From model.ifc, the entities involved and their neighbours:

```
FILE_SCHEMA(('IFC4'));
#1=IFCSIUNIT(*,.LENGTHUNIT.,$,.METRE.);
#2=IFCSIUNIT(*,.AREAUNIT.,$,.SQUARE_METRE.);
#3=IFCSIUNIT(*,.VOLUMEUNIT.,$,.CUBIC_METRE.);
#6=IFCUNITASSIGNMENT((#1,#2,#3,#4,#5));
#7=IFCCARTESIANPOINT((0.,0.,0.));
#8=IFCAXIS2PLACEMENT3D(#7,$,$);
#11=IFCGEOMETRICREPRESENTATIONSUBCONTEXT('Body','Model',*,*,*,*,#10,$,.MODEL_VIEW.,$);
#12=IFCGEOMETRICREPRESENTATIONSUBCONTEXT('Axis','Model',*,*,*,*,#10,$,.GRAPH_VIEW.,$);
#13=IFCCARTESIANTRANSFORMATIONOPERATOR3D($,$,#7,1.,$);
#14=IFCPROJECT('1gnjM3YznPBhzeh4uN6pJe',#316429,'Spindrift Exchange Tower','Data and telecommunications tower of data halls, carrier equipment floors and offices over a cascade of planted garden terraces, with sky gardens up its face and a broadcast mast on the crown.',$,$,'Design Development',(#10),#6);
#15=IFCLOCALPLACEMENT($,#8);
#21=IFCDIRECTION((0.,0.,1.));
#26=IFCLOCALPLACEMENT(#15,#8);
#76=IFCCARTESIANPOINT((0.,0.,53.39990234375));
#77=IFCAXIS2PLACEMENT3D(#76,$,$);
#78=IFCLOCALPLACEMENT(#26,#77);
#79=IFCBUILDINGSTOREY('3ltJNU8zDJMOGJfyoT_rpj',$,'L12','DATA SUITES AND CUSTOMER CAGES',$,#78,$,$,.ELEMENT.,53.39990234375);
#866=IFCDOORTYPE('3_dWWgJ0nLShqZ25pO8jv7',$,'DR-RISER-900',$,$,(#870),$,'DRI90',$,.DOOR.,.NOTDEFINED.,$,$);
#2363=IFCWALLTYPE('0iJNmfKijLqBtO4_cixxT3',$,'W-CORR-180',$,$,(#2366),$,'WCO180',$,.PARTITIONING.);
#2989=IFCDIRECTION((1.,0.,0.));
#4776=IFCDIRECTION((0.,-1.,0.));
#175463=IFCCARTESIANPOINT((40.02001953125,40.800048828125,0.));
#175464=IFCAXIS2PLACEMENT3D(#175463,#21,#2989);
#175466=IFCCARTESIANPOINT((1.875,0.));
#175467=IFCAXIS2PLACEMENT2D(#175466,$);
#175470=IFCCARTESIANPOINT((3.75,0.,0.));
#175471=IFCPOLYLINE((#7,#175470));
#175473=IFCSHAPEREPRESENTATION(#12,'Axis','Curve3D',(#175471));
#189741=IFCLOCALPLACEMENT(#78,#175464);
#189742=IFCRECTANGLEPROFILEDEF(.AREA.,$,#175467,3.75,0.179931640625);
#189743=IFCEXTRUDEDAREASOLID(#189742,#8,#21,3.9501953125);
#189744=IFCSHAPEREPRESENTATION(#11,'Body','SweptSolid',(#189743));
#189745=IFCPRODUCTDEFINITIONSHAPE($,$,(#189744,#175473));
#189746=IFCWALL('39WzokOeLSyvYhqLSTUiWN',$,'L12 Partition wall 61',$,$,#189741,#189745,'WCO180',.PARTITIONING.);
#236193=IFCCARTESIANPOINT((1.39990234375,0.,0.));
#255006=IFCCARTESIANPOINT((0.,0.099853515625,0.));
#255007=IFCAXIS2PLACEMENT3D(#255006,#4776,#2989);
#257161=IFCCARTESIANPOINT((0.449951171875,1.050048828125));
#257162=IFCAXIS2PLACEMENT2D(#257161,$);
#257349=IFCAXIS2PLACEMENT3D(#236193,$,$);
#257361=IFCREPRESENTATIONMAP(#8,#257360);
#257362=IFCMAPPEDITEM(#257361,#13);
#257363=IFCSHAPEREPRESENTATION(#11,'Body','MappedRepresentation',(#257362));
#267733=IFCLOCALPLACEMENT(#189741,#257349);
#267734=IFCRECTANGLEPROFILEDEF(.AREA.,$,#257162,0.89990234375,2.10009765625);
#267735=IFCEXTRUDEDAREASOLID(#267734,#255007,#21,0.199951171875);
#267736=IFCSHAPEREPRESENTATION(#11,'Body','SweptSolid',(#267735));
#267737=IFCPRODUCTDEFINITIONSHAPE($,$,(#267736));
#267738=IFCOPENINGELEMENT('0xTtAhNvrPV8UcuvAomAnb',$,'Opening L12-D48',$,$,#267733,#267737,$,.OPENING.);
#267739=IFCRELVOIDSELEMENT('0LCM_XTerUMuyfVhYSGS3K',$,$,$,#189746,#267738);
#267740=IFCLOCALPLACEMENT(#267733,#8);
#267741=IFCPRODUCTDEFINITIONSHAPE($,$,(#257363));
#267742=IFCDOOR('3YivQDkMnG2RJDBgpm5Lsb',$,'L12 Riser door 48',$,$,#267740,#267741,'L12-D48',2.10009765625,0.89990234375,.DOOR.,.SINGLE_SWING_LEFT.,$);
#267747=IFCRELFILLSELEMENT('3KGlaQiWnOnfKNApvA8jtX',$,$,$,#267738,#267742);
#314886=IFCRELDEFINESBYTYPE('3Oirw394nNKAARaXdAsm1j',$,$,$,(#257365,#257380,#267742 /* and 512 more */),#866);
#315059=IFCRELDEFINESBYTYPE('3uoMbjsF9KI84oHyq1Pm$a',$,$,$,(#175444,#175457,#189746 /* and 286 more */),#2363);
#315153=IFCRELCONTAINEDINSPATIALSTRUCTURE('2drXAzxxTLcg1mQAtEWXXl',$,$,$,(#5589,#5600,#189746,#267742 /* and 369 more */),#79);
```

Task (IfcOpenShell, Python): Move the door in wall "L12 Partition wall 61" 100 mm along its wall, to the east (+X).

```python
import ifcopenshell
import ifcopenshell.api.geometry
import ifcopenshell.util.placement

model = ifcopenshell.open("model.ifc")

door = model.by_guid("3YivQDkMnG2RJDBgpm5Lsb")
opening = door.FillsVoids[0].RelatingOpeningElement
wall = opening.VoidsElements[0].RelatingBuildingElement

wall_matrix = ifcopenshell.util.placement.get_local_placement(wall.ObjectPlacement)
shift = wall_matrix[:3, 0] * 0.1
before = ifcopenshell.util.placement.get_local_placement(door.ObjectPlacement)[:3, 3].copy()

# The door is placed relative to its opening, so it follows when the opening moves.
matrix = ifcopenshell.util.placement.get_local_placement(opening.ObjectPlacement)
matrix[:3, 3] += shift
ifcopenshell.api.geometry.edit_object_placement(
    model, product=opening, matrix=matrix, is_si=False, should_transform_children=True
)

after = ifcopenshell.util.placement.get_local_placement(door.ObjectPlacement)[:3, 3]
print("door moved by", (after - before).round(3) + 0.0)

model.write("model-out.ifc")
```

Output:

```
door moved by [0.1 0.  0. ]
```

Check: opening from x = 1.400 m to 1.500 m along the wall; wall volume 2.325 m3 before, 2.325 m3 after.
